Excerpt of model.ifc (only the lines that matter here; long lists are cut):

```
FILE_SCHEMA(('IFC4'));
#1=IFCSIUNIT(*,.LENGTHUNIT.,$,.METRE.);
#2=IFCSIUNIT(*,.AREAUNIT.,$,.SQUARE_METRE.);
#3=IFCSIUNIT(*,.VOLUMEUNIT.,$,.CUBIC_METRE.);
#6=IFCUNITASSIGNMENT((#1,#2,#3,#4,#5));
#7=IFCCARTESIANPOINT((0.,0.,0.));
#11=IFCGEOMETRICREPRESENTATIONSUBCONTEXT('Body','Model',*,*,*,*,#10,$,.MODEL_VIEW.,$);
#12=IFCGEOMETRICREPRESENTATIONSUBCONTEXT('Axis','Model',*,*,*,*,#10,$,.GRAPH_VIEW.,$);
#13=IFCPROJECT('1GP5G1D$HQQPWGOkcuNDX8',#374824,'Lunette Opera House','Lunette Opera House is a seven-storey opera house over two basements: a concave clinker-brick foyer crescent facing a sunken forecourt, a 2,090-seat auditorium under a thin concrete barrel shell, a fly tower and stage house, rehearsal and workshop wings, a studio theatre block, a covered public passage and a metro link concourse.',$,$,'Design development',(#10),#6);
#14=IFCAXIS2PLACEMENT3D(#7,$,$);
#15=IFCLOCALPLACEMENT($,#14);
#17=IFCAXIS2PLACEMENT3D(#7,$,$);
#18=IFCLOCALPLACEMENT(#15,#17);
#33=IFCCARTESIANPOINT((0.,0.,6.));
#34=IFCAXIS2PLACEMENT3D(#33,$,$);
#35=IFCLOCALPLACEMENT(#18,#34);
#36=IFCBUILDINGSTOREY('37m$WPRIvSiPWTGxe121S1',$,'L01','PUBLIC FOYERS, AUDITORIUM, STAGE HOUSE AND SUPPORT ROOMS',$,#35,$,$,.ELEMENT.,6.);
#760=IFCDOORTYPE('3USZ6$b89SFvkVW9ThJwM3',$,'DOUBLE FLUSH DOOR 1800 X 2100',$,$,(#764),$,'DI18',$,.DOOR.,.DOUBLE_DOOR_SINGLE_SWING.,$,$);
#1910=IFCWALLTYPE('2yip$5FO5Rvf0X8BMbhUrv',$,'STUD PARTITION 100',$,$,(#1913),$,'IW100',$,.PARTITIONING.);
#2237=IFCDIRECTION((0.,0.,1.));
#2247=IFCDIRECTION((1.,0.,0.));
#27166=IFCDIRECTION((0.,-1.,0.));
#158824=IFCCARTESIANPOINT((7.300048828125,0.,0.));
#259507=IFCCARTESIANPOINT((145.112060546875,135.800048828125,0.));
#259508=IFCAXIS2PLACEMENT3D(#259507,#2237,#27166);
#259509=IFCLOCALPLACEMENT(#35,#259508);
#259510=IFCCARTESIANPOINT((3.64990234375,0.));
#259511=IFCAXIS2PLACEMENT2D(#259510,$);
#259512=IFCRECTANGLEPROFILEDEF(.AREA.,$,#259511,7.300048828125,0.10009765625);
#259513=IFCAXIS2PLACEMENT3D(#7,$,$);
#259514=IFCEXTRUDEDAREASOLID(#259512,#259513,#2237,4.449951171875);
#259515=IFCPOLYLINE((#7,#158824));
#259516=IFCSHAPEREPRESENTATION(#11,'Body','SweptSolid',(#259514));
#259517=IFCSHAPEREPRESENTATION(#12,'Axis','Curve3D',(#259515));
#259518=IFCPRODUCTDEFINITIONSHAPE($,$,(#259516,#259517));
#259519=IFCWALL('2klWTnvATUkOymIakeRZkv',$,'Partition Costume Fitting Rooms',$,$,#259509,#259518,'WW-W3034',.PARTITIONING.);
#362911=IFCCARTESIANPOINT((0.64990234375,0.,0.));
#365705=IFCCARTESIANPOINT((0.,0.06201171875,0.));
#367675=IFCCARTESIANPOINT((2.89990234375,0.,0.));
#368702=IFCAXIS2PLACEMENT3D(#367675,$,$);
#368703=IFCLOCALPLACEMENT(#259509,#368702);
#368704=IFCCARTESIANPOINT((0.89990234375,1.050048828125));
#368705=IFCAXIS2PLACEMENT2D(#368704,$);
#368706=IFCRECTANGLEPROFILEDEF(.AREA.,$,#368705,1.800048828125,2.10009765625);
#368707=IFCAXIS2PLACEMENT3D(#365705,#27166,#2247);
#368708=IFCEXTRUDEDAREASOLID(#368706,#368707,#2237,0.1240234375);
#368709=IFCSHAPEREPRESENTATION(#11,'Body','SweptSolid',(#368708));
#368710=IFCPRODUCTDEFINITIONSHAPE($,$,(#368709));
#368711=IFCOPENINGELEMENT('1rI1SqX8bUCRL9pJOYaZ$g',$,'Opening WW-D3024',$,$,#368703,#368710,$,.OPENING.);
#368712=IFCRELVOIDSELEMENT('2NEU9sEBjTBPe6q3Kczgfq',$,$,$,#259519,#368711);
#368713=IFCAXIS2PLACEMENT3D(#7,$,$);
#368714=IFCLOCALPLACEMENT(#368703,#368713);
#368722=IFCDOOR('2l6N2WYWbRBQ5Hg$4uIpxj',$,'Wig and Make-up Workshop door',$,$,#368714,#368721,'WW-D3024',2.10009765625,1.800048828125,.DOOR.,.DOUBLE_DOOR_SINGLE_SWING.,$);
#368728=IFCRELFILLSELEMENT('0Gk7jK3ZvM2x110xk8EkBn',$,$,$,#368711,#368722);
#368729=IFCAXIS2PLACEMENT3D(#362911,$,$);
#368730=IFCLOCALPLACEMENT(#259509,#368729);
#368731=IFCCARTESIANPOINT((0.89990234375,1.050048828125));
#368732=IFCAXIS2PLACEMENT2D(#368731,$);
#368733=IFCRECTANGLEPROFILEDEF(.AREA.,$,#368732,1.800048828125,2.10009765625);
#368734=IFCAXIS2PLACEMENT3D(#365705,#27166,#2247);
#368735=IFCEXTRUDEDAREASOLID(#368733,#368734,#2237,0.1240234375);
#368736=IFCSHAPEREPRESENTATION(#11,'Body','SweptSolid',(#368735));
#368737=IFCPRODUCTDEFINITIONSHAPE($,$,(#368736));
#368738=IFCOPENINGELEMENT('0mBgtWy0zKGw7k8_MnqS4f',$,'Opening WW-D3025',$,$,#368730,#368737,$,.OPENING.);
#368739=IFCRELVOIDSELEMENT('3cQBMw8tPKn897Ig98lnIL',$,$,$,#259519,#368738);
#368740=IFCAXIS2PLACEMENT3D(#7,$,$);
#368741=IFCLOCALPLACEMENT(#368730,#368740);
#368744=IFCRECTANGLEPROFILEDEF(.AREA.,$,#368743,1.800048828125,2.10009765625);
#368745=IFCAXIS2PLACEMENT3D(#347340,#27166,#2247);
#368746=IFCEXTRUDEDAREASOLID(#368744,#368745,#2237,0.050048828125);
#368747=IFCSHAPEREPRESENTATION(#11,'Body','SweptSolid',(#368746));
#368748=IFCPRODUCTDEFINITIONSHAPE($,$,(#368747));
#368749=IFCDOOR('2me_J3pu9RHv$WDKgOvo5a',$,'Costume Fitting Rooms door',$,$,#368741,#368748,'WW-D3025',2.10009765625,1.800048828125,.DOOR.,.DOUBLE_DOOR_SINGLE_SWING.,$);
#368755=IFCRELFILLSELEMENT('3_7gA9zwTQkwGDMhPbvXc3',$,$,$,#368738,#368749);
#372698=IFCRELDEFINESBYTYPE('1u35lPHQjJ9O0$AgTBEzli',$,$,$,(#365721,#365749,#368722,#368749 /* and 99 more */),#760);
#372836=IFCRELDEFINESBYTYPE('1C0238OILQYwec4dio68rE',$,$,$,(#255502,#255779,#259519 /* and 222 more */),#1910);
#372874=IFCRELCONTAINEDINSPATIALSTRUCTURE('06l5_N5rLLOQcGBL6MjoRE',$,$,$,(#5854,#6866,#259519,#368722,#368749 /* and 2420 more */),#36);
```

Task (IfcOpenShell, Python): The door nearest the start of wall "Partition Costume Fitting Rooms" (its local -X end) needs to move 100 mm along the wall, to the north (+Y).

```python
import ifcopenshell
import ifcopenshell.api.geometry
import ifcopenshell.util.placement
import ifcopenshell.util.unit

model = ifcopenshell.open("model.ifc")
unit_scale = ifcopenshell.util.unit.calculate_unit_scale(model)

door = model.by_guid("2me_J3pu9RHv$WDKgOvo5a")
opening = door.FillsVoids[0].RelatingOpeningElement
wall = opening.VoidsElements[0].RelatingBuildingElement

wall_matrix = ifcopenshell.util.placement.get_local_placement(wall.ObjectPlacement)
shift = wall_matrix[:3, 0] * -0.1 / unit_scale
before = ifcopenshell.util.placement.get_local_placement(door.ObjectPlacement)[:3, 3].copy()

# The door is placed relative to its opening, so it follows when the opening moves.
matrix = ifcopenshell.util.placement.get_local_placement(opening.ObjectPlacement)
matrix[:3, 3] += shift
ifcopenshell.api.geometry.edit_object_placement(
    model, product=opening, matrix=matrix, is_si=False, should_transform_children=True
)

after = ifcopenshell.util.placement.get_local_placement(door.ObjectPlacement)[:3, 3]
print("door moved by", (after - before).round(3) + 0.0)

model.write("model_updated.ifc")
```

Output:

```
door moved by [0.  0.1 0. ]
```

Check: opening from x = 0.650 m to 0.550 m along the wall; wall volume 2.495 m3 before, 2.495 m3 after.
